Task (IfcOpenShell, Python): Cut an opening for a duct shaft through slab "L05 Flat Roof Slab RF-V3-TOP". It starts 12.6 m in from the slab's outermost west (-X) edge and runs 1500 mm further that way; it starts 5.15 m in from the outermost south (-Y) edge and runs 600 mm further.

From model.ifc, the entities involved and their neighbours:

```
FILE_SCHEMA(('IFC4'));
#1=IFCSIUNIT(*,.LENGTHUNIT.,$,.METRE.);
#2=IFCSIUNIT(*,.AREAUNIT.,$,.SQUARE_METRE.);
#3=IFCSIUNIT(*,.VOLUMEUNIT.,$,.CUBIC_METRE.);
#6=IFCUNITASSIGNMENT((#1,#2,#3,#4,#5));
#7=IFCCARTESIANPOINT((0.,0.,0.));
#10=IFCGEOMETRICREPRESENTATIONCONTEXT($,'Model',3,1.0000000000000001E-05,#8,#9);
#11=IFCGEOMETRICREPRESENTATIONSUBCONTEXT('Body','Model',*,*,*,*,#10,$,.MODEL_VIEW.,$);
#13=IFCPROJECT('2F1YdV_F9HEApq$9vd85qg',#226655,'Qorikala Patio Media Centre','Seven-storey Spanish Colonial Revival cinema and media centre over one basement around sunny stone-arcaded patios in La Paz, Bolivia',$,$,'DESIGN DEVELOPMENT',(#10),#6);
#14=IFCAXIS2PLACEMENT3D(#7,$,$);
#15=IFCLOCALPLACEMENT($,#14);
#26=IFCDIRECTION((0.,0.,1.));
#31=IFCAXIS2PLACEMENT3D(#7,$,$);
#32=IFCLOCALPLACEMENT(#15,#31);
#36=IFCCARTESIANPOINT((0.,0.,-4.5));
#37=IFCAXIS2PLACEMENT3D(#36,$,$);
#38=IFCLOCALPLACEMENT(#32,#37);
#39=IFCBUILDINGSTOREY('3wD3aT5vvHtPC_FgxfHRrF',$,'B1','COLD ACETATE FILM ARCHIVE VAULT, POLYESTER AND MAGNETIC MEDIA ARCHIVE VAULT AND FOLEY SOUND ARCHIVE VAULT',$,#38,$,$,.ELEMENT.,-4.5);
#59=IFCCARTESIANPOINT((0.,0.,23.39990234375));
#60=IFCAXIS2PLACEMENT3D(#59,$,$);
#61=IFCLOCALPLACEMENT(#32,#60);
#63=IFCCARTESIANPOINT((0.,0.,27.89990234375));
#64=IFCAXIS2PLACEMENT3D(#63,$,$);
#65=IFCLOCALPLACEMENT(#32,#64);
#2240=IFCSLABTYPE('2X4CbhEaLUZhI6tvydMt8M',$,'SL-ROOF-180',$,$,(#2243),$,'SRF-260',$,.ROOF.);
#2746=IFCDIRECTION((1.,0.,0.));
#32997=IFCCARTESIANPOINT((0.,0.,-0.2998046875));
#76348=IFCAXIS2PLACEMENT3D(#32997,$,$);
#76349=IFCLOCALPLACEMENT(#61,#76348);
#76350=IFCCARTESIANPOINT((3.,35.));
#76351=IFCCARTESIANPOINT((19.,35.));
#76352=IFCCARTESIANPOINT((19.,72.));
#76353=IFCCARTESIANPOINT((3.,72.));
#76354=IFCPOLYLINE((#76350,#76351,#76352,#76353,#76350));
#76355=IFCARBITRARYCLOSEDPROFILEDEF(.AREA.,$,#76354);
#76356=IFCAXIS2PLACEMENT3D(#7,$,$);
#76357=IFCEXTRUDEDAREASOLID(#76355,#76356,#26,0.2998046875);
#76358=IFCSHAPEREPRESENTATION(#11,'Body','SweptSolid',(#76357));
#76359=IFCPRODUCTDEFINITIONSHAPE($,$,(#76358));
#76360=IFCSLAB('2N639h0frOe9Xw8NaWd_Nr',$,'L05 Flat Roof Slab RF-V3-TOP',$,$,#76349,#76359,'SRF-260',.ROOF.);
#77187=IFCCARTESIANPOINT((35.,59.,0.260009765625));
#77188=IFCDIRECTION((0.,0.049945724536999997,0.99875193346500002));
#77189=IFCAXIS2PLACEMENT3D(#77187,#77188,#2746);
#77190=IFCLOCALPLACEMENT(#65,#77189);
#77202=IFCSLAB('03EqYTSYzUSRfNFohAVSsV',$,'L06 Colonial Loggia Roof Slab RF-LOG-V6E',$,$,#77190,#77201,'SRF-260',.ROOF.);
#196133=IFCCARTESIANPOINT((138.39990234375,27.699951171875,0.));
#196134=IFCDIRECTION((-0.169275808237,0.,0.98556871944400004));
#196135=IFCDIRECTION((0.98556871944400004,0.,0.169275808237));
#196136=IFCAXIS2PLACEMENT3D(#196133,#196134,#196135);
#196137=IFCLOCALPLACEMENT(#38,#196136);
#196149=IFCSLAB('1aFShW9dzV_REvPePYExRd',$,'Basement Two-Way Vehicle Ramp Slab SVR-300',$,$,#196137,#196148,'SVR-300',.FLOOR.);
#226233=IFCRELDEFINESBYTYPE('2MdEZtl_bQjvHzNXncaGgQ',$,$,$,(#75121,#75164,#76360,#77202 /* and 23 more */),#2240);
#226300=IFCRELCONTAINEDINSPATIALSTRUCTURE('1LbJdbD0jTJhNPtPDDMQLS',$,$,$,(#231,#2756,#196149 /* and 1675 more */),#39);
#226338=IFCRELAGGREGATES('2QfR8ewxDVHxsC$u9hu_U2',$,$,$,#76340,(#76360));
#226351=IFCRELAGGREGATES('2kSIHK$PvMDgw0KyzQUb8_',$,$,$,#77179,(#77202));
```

```python
import numpy as np
import ifcopenshell
import ifcopenshell.api.feature
import ifcopenshell.api.geometry
import ifcopenshell.api.root
import ifcopenshell.geom
import ifcopenshell.util.placement
import ifcopenshell.util.representation
import ifcopenshell.util.shape
import ifcopenshell.util.unit

model = ifcopenshell.open("model.ifc")
unit_scale = ifcopenshell.util.unit.calculate_unit_scale(model)
settings = ifcopenshell.geom.settings()


def volume(element):
    """Net volume in cubic metres, openings subtracted."""
    shape = ifcopenshell.geom.create_shape(settings, element)
    return ifcopenshell.util.shape.get_volume(shape.geometry)


slab = model.by_guid("2N639h0frOe9Xw8NaWd_Nr")
before = volume(slab)

# Extent in the slab's own axes, in metres. The edges named are its -X and -Y sides.
slab_shape = ifcopenshell.geom.create_shape(settings, slab)
vertices = ifcopenshell.util.shape.get_vertices(slab_shape.geometry)
x_min, y_min, bottom = vertices.min(axis=0)
top = vertices[:, 2].max()

opening = ifcopenshell.api.root.create_entity(model, ifc_class="IfcOpeningElement", name="Duct shaft opening", predefined_type="OPENING")
context = ifcopenshell.util.representation.get_context(model, "Model", "Body", "MODEL_VIEW")
width, depth = 1.5, 0.6
outline = [(0.0, 0.0), (width, 0.0), (width, depth), (0.0, depth), (0.0, 0.0)]
# Overshoot both faces by 50 mm so the cut is clean.
shape = ifcopenshell.api.geometry.add_slab_representation(
    model, context=context, depth=top - bottom + 0.1, polyline=outline
)
ifcopenshell.api.geometry.assign_representation(model, product=opening, representation=shape)

matrix = ifcopenshell.util.placement.get_local_placement(slab.ObjectPlacement)
matrix[:, 3] = matrix @ np.append(np.array([x_min + 12.6, y_min + 5.15, bottom - 0.05]) / unit_scale, 1.0)
ifcopenshell.api.geometry.edit_object_placement(model, product=opening, matrix=matrix, is_si=False)
ifcopenshell.api.feature.add_feature(model, feature=opening, element=slab)

after = volume(slab)

print(f"slab volume {before:.3f} -> {after:.3f} m3")

model.write("model_edited.ifc")
```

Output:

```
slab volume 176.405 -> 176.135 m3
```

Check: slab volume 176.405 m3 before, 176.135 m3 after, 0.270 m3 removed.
